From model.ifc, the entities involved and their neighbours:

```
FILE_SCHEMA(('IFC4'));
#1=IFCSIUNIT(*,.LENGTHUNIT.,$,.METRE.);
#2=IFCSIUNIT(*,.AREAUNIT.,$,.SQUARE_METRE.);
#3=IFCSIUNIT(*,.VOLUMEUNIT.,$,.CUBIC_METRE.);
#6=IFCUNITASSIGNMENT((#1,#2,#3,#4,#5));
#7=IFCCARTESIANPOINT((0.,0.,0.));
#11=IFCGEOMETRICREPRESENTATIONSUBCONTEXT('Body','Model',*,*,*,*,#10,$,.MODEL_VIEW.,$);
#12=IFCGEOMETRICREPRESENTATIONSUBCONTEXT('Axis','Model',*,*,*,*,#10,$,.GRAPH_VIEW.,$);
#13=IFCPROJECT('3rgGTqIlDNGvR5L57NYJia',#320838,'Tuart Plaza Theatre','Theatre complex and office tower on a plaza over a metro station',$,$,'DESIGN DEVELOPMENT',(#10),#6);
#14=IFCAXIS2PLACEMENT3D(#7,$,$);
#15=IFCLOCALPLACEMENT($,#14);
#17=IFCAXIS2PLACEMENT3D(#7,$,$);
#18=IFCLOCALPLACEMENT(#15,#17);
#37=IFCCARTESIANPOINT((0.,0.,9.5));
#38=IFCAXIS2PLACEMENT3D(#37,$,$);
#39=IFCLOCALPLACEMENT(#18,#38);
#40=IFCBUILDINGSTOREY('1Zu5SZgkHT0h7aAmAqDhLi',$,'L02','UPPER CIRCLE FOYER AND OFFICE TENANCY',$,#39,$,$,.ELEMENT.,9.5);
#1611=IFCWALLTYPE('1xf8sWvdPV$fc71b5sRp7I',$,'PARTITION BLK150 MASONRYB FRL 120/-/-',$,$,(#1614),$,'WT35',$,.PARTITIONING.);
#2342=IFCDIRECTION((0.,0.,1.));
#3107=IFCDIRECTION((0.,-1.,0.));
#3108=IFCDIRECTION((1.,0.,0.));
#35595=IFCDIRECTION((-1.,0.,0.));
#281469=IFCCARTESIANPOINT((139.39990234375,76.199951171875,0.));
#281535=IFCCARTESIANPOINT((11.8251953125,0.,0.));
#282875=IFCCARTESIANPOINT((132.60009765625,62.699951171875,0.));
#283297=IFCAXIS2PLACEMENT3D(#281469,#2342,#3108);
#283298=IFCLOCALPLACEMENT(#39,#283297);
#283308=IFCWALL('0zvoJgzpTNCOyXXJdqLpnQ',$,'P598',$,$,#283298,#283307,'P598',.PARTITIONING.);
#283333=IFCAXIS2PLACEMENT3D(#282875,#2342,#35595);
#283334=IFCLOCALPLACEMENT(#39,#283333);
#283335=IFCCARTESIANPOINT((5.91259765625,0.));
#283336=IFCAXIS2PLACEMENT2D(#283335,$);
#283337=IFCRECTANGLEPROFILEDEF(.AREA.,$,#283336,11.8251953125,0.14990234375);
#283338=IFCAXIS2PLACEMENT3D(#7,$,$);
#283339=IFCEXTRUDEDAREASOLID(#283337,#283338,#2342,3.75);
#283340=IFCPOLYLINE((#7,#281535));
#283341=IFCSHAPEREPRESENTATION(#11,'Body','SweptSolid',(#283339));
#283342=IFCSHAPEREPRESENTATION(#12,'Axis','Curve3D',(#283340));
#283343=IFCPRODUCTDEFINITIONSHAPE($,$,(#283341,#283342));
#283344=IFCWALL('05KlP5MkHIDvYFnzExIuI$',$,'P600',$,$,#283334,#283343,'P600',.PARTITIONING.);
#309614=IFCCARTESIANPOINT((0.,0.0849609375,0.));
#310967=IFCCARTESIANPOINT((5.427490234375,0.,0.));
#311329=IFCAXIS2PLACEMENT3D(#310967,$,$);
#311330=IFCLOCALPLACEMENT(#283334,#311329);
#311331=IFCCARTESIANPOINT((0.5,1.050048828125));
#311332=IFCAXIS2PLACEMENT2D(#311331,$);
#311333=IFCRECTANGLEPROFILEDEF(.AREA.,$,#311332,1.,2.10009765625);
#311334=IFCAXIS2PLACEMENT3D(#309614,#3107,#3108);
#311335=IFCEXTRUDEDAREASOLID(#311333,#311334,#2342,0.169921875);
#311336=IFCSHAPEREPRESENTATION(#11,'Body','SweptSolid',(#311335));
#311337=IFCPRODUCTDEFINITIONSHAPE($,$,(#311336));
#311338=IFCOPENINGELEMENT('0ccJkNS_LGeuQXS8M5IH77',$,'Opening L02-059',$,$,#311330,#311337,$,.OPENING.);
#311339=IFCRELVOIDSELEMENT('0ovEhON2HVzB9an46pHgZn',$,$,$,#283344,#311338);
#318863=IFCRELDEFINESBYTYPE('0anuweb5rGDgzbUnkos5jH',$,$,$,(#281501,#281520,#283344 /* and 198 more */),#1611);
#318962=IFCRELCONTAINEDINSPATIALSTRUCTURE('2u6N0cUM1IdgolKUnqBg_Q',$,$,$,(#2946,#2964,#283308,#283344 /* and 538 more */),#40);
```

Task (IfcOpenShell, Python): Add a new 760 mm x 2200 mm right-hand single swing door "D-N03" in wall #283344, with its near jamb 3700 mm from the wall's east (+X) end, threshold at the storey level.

```python
import numpy as np
import ifcopenshell
import ifcopenshell.api.feature
import ifcopenshell.api.geometry
import ifcopenshell.api.root
import ifcopenshell.api.spatial
import ifcopenshell.geom
import ifcopenshell.util.element
import ifcopenshell.util.placement
import ifcopenshell.util.representation
import ifcopenshell.util.shape
import ifcopenshell.util.unit

model = ifcopenshell.open("model.ifc")
unit_scale = ifcopenshell.util.unit.calculate_unit_scale(model)
settings = ifcopenshell.geom.settings()


def volume(element):
    """Net volume in cubic metres, openings subtracted."""
    shape = ifcopenshell.geom.create_shape(settings, element)
    return ifcopenshell.util.shape.get_volume(shape.geometry)


wall = model.by_guid("05KlP5MkHIDvYFnzExIuI$")
storey = ifcopenshell.util.element.get_container(wall, ifc_class="IfcBuildingStorey")
context = ifcopenshell.util.representation.get_context(model, "Model", "Body", "MODEL_VIEW")
before = volume(wall)

width, height, from_end, sill = 0.76, 2.2, 3.7, 0.0  # metres

# The wall runs along its own X axis, and the end named is its -X end.
wall_shape = ifcopenshell.geom.create_shape(settings, wall)
x, y, z = ifcopenshell.util.shape.get_vertices(wall_shape.geometry).T
start = x.min() + from_end
face, thickness = float(y.min()), float(y.max() - y.min())
wall_matrix = ifcopenshell.util.placement.get_local_placement(wall.ObjectPlacement)
level = ifcopenshell.util.placement.get_local_placement(storey.ObjectPlacement)[2, 3]


def in_wall(x, y):
    """Placement at x, y metres in the wall's axes, at sill height."""
    matrix = wall_matrix.copy()
    matrix[:, 3] = wall_matrix @ np.array([x / unit_scale, y / unit_scale, 0.0, 1.0])
    matrix[2, 3] = level + sill / unit_scale
    return matrix


# Opening: a box that overshoots both wall faces by 50 mm.
opening = ifcopenshell.api.root.create_entity(model, ifc_class="IfcOpeningElement", predefined_type="OPENING")
box = ifcopenshell.api.geometry.add_wall_representation(
    model, context=context, length=width, height=height, thickness=thickness + 0.1
)
ifcopenshell.api.geometry.assign_representation(model, product=opening, representation=box)
ifcopenshell.api.geometry.edit_object_placement(model, product=opening, matrix=in_wall(start, face - 0.05), is_si=False)
ifcopenshell.api.feature.add_feature(model, feature=opening, element=wall)

door = ifcopenshell.api.root.create_entity(model, ifc_class="IfcDoor", name="D-N03", predefined_type="DOOR")
door.OverallWidth, door.OverallHeight = width / unit_scale, height / unit_scale
door.OperationType = "SINGLE_SWING_RIGHT"
body = ifcopenshell.api.geometry.add_door_representation(
    model,
    context=context,
    overall_width=door.OverallWidth,
    overall_height=door.OverallHeight,
    operation_type="SINGLE_SWING_RIGHT",
    lining_properties={"LiningDepth": thickness / unit_scale, "ThresholdDepth": thickness / unit_scale},
)
ifcopenshell.api.geometry.assign_representation(model, product=door, representation=body)
ifcopenshell.api.spatial.assign_container(model, products=[door], relating_structure=storey)
ifcopenshell.api.feature.add_filling(model, opening=opening, element=door)

# The lining spans the wall, so the door starts at the wall face.
ifcopenshell.api.geometry.edit_object_placement(model, product=door, matrix=in_wall(start, face), is_si=False)

after = volume(wall)

print(f"wall volume {before:.3f} -> {after:.3f} m3")

model.write("model_rev.ifc")
```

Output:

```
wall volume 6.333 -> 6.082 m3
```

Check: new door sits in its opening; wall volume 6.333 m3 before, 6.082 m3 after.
